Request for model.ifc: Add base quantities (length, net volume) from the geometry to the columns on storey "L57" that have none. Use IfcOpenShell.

First a look at what the model holds.

```python
import ifcopenshell
import ifcopenshell.util.element
import ifcopenshell.util.unit

model = ifcopenshell.open("model.ifc")
print(model.schema)
for unit_type in ("LENGTHUNIT", "AREAUNIT", "VOLUMEUNIT"):
    print(unit_type, ifcopenshell.util.unit.calculate_unit_scale(model, unit_type))
storey = next(s for s in model.by_type("IfcBuildingStorey") if s.Name == "L57")
columns = [e for e in ifcopenshell.util.element.get_decomposition(storey) if e.is_a("IfcColumn")]
for e in sorted(columns, key=lambda e: e.id()):
    print(e.id(), e.is_a(), e.Name, list(ifcopenshell.util.element.get_psets(e, qtos_only=True)), sep=" | ")
```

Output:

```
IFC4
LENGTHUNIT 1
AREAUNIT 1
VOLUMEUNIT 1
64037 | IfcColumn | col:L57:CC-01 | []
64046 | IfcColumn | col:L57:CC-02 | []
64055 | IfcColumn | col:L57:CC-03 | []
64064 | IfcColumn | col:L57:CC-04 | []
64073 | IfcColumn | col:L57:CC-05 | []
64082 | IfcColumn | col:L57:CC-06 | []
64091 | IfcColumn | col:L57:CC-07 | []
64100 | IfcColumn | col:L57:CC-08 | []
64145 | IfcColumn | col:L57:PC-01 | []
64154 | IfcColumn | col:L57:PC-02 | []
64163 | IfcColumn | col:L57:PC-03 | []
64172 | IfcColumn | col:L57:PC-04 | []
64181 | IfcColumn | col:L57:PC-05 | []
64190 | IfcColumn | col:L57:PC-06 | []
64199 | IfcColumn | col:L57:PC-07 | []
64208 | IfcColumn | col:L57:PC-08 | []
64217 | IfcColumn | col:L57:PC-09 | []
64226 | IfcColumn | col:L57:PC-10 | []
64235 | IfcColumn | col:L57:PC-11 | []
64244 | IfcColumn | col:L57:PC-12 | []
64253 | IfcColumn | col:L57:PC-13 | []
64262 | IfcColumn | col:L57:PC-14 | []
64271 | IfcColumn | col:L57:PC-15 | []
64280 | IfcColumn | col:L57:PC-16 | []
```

```python
import ifcopenshell
import ifcopenshell.api.pset
import ifcopenshell.geom
import ifcopenshell.util.element
import ifcopenshell.util.shape
import ifcopenshell.util.unit

model = ifcopenshell.open("model.ifc")
unit_scale = ifcopenshell.util.unit.calculate_unit_scale(model)
volume_scale = ifcopenshell.util.unit.calculate_unit_scale(model, "VOLUMEUNIT")
settings = ifcopenshell.geom.settings()

storey = next(s for s in model.by_type("IfcBuildingStorey") if s.Name == "L57")
columns = [e for e in ifcopenshell.util.element.get_decomposition(storey) if e.is_a("IfcColumn")]

for e in sorted(columns, key=lambda e: e.id()):
    if ifcopenshell.util.element.get_psets(e, qtos_only=True, should_inherit=False):
        continue
    # Geometry comes back in metres, in the element's own axes.
    shape = ifcopenshell.geom.create_shape(settings, e)
    values = {
        "Length": ifcopenshell.util.shape.get_z(shape.geometry) / unit_scale,
        "NetVolume": ifcopenshell.util.shape.get_volume(shape.geometry) / volume_scale,
    }
    qto = ifcopenshell.api.pset.add_qto(model, product=e, name="Qto_ColumnBaseQuantities")
    ifcopenshell.api.pset.edit_qto(model, qto=qto, properties=values)
    print(e.id(), {k: round(v, 3) for k, v in values.items()})

model.write("model_v2.ifc")
```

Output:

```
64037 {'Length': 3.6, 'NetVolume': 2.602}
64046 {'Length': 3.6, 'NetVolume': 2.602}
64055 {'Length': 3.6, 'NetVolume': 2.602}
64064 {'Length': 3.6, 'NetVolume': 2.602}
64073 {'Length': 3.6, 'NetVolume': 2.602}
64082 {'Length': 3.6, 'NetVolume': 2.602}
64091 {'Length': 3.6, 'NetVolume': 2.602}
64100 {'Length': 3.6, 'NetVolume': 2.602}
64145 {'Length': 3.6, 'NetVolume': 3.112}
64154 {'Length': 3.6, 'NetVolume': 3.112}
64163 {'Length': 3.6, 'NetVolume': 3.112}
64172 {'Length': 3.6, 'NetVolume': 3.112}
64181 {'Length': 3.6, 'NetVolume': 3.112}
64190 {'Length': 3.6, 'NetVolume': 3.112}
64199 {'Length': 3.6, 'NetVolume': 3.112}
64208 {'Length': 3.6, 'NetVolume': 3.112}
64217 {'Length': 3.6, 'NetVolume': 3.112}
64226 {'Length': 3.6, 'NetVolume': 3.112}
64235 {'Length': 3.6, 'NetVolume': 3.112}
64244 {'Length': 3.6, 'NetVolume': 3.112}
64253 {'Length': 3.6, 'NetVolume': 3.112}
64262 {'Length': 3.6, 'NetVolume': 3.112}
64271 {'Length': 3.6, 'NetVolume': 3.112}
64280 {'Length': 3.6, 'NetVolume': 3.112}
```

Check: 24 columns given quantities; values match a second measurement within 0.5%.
